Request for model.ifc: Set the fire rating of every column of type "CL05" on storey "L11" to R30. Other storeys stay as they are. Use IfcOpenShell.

First a look at what the model holds.

```python
import ifcopenshell
import ifcopenshell.util.element

model = ifcopenshell.open("model.ifc")
print(model.schema)
storey = next(s for s in model.by_type("IfcBuildingStorey") if s.Name == "L11")
columns = [e for e in ifcopenshell.util.element.get_decomposition(storey) if e.is_a("IfcColumn")]
seen = {}
for e in columns:
    element_type = ifcopenshell.util.element.get_type(e)
    key = (element_type.Name if element_type != e and element_type else None, ifcopenshell.util.element.get_pset(e, "Pset_ColumnCommon", "FireRating"))
    seen[key] = seen.get(key, 0) + 1
for (name, value), count in sorted(seen.items(), key=str):
    print(count, "x", name, "|", value)
```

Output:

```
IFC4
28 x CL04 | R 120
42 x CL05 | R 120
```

```python
import ifcopenshell
import ifcopenshell.api.pset
import ifcopenshell.util.element

model = ifcopenshell.open("model.ifc")

storey = next(s for s in model.by_type("IfcBuildingStorey") if s.Name == "L11")
columns = [e for e in ifcopenshell.util.element.get_decomposition(storey) if e.is_a("IfcColumn")]

count = 0
for e in columns:
    element_type = ifcopenshell.util.element.get_type(e)
    if element_type in (None, e) or element_type.Name != "CL05":
        continue
    # add_pset returns the element's existing set when there is one.
    pset = ifcopenshell.api.pset.add_pset(model, product=e, name="Pset_ColumnCommon")
    ifcopenshell.api.pset.edit_pset(model, pset=pset, properties={"FireRating": "R30"})
    count += 1

print(count, "columns updated")

model.write("model-out.ifc")
```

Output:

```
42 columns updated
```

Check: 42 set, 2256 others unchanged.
